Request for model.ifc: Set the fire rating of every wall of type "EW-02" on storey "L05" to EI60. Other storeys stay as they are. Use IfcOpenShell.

First a look at what the model holds.

```python
import ifcopenshell
import ifcopenshell.util.element

model = ifcopenshell.open("model.ifc")
print(model.schema)
storey = next(s for s in model.by_type("IfcBuildingStorey") if s.Name == "L05")
walls = [e for e in ifcopenshell.util.element.get_decomposition(storey) if e.is_a("IfcWall")]
seen = {}
for e in walls:
    element_type = ifcopenshell.util.element.get_type(e)
    key = (element_type.Name if element_type != e and element_type else None, ifcopenshell.util.element.get_pset(e, "Pset_WallCommon", "FireRating"))
    seen[key] = seen.get(key, 0) + 1
for (name, value), count in sorted(seen.items(), key=str):
    print(count, "x", name, "|", value)
```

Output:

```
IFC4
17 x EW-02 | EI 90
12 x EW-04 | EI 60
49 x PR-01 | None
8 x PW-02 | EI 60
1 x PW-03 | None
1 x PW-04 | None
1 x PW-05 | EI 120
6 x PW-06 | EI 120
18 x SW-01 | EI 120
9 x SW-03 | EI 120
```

```python
import ifcopenshell
import ifcopenshell.api.pset
import ifcopenshell.util.element

model = ifcopenshell.open("model.ifc")

storey = next(s for s in model.by_type("IfcBuildingStorey") if s.Name == "L05")
walls = [e for e in ifcopenshell.util.element.get_decomposition(storey) if e.is_a("IfcWall")]

count = 0
for e in walls:
    element_type = ifcopenshell.util.element.get_type(e)
    if element_type in (None, e) or element_type.Name != "EW-02":
        continue
    # add_pset returns the element's existing set when there is one.
    pset = ifcopenshell.api.pset.add_pset(model, product=e, name="Pset_WallCommon")
    ifcopenshell.api.pset.edit_pset(model, pset=pset, properties={"FireRating": "EI60"})
    count += 1

print(count, "walls updated")

model.write("model_rev.ifc")
```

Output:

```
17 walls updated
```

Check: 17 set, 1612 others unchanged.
